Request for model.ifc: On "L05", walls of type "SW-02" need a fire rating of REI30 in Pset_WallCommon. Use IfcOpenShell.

First a look at what the model holds.

```python
import ifcopenshell
import ifcopenshell.util.element

model = ifcopenshell.open("model.ifc")
print(model.schema)
storey = next(s for s in model.by_type("IfcBuildingStorey") if s.Name == "L05")
walls = [e for e in ifcopenshell.util.element.get_decomposition(storey) if e.is_a("IfcWall")]
seen = {}
for e in walls:
    element_type = ifcopenshell.util.element.get_type(e)
    key = (element_type.Name if element_type != e and element_type else None, ifcopenshell.util.element.get_pset(e, "Pset_WallCommon", "FireRating"))
    seen[key] = seen.get(key, 0) + 1
for (name, value), count in sorted(seen.items(), key=str):
    print(count, "x", name, "|", value)
```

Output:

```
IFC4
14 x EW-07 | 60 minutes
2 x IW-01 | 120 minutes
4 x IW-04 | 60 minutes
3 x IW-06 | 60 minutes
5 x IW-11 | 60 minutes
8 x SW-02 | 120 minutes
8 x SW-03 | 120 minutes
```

```python
import ifcopenshell
import ifcopenshell.api.pset
import ifcopenshell.util.element

model = ifcopenshell.open("model.ifc")

storey = next(s for s in model.by_type("IfcBuildingStorey") if s.Name == "L05")
walls = [e for e in ifcopenshell.util.element.get_decomposition(storey) if e.is_a("IfcWall")]

count = 0
for e in walls:
    element_type = ifcopenshell.util.element.get_type(e)
    if element_type in (None, e) or element_type.Name != "SW-02":
        continue
    # add_pset returns the element's existing set when there is one.
    pset = ifcopenshell.api.pset.add_pset(model, product=e, name="Pset_WallCommon")
    ifcopenshell.api.pset.edit_pset(model, pset=pset, properties={"FireRating": "REI30"})
    count += 1

print(count, "walls updated")

model.write("model-out.ifc")
```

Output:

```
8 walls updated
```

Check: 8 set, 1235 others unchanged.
